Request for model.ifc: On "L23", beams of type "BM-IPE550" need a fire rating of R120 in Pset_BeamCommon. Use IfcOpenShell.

First a look at what the model holds.

```python
import ifcopenshell
import ifcopenshell.util.element

model = ifcopenshell.open("model.ifc")
print(model.schema)
storey = next(s for s in model.by_type("IfcBuildingStorey") if s.Name == "L23")
beams = [e for e in ifcopenshell.util.element.get_decomposition(storey) if e.is_a("IfcBeam")]
seen = {}
for e in beams:
    element_type = ifcopenshell.util.element.get_type(e)
    key = (element_type.Name if element_type != e and element_type else None, ifcopenshell.util.element.get_pset(e, "Pset_BeamCommon", "FireRating"))
    seen[key] = seen.get(key, 0) + 1
for (name, value), count in sorted(seen.items(), key=str):
    print(count, "x", name, "|", value)
```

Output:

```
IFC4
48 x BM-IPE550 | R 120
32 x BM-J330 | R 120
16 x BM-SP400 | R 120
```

```python
import ifcopenshell
import ifcopenshell.api.pset
import ifcopenshell.util.element

model = ifcopenshell.open("model.ifc")

storey = next(s for s in model.by_type("IfcBuildingStorey") if s.Name == "L23")
beams = [e for e in ifcopenshell.util.element.get_decomposition(storey) if e.is_a("IfcBeam")]

count = 0
for e in beams:
    element_type = ifcopenshell.util.element.get_type(e)
    if element_type in (None, e) or element_type.Name != "BM-IPE550":
        continue
    # add_pset returns the element's existing set when there is one.
    pset = ifcopenshell.api.pset.add_pset(model, product=e, name="Pset_BeamCommon")
    ifcopenshell.api.pset.edit_pset(model, pset=pset, properties={"FireRating": "R120"})
    count += 1

print(count, "beams updated")

model.write("model-out.ifc")
```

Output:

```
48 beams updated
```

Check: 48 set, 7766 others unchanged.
